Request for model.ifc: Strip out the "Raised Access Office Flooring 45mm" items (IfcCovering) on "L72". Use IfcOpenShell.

First a look at what the model holds.

```python
import ifcopenshell
import ifcopenshell.util.element

model = ifcopenshell.open("model.ifc")
print(model.schema)
storey = next(s for s in model.by_type("IfcBuildingStorey") if s.Name == "L72")
coverings = [e for e in ifcopenshell.util.element.get_decomposition(storey) if e.is_a("IfcCovering")]
seen = {}
for e in coverings:
    element_type = ifcopenshell.util.element.get_type(e)
    name = element_type.Name if element_type not in (None, e) else None
    seen[name] = seen.get(name, 0) + 1
for name, count in sorted(seen.items(), key=str):
    print(count, "x", name)
```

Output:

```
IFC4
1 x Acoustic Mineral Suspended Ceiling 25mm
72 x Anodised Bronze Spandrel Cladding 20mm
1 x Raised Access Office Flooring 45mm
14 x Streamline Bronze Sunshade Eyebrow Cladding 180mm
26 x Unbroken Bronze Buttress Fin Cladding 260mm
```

```python
import ifcopenshell
import ifcopenshell.api.root
import ifcopenshell.util.element

model = ifcopenshell.open("model.ifc")

storey = next(s for s in model.by_type("IfcBuildingStorey") if s.Name == "L72")
coverings = [e for e in ifcopenshell.util.element.get_decomposition(storey) if e.is_a("IfcCovering")]
targets = [e for e in coverings if (t := ifcopenshell.util.element.get_type(e)) not in (None, e) and t.Name == "Raised Access Office Flooring 45mm"]

for e in targets:
    ifcopenshell.api.root.remove_product(model, product=e)
print(len(targets), "removed")

model.write("model_updated.ifc")
```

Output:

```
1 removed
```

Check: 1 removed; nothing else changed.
